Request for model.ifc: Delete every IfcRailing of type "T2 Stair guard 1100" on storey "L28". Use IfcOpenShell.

First a look at what the model holds.

```python
import ifcopenshell
import ifcopenshell.util.element

model = ifcopenshell.open("model.ifc")
print(model.schema)
storey = next(s for s in model.by_type("IfcBuildingStorey") if s.Name == "L28")
railings = [e for e in ifcopenshell.util.element.get_decomposition(storey) if e.is_a("IfcRailing")]
seen = {}
for e in railings:
    element_type = ifcopenshell.util.element.get_type(e)
    name = element_type.Name if element_type not in (None, e) else None
    seen[name] = seen.get(name, 0) + 1
for name, count in sorted(seen.items(), key=str):
    print(count, "x", name)
```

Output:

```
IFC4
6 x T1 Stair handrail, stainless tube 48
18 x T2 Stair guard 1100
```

```python
import ifcopenshell
import ifcopenshell.api.root
import ifcopenshell.util.element

model = ifcopenshell.open("model.ifc")

storey = next(s for s in model.by_type("IfcBuildingStorey") if s.Name == "L28")
railings = [e for e in ifcopenshell.util.element.get_decomposition(storey) if e.is_a("IfcRailing")]
targets = [e for e in railings if (t := ifcopenshell.util.element.get_type(e)) not in (None, e) and t.Name == "T2 Stair guard 1100"]

for e in targets:
    ifcopenshell.api.root.remove_product(model, product=e)
print(len(targets), "removed")

model.write("model_rev.ifc")
```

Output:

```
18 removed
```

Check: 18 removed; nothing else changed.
